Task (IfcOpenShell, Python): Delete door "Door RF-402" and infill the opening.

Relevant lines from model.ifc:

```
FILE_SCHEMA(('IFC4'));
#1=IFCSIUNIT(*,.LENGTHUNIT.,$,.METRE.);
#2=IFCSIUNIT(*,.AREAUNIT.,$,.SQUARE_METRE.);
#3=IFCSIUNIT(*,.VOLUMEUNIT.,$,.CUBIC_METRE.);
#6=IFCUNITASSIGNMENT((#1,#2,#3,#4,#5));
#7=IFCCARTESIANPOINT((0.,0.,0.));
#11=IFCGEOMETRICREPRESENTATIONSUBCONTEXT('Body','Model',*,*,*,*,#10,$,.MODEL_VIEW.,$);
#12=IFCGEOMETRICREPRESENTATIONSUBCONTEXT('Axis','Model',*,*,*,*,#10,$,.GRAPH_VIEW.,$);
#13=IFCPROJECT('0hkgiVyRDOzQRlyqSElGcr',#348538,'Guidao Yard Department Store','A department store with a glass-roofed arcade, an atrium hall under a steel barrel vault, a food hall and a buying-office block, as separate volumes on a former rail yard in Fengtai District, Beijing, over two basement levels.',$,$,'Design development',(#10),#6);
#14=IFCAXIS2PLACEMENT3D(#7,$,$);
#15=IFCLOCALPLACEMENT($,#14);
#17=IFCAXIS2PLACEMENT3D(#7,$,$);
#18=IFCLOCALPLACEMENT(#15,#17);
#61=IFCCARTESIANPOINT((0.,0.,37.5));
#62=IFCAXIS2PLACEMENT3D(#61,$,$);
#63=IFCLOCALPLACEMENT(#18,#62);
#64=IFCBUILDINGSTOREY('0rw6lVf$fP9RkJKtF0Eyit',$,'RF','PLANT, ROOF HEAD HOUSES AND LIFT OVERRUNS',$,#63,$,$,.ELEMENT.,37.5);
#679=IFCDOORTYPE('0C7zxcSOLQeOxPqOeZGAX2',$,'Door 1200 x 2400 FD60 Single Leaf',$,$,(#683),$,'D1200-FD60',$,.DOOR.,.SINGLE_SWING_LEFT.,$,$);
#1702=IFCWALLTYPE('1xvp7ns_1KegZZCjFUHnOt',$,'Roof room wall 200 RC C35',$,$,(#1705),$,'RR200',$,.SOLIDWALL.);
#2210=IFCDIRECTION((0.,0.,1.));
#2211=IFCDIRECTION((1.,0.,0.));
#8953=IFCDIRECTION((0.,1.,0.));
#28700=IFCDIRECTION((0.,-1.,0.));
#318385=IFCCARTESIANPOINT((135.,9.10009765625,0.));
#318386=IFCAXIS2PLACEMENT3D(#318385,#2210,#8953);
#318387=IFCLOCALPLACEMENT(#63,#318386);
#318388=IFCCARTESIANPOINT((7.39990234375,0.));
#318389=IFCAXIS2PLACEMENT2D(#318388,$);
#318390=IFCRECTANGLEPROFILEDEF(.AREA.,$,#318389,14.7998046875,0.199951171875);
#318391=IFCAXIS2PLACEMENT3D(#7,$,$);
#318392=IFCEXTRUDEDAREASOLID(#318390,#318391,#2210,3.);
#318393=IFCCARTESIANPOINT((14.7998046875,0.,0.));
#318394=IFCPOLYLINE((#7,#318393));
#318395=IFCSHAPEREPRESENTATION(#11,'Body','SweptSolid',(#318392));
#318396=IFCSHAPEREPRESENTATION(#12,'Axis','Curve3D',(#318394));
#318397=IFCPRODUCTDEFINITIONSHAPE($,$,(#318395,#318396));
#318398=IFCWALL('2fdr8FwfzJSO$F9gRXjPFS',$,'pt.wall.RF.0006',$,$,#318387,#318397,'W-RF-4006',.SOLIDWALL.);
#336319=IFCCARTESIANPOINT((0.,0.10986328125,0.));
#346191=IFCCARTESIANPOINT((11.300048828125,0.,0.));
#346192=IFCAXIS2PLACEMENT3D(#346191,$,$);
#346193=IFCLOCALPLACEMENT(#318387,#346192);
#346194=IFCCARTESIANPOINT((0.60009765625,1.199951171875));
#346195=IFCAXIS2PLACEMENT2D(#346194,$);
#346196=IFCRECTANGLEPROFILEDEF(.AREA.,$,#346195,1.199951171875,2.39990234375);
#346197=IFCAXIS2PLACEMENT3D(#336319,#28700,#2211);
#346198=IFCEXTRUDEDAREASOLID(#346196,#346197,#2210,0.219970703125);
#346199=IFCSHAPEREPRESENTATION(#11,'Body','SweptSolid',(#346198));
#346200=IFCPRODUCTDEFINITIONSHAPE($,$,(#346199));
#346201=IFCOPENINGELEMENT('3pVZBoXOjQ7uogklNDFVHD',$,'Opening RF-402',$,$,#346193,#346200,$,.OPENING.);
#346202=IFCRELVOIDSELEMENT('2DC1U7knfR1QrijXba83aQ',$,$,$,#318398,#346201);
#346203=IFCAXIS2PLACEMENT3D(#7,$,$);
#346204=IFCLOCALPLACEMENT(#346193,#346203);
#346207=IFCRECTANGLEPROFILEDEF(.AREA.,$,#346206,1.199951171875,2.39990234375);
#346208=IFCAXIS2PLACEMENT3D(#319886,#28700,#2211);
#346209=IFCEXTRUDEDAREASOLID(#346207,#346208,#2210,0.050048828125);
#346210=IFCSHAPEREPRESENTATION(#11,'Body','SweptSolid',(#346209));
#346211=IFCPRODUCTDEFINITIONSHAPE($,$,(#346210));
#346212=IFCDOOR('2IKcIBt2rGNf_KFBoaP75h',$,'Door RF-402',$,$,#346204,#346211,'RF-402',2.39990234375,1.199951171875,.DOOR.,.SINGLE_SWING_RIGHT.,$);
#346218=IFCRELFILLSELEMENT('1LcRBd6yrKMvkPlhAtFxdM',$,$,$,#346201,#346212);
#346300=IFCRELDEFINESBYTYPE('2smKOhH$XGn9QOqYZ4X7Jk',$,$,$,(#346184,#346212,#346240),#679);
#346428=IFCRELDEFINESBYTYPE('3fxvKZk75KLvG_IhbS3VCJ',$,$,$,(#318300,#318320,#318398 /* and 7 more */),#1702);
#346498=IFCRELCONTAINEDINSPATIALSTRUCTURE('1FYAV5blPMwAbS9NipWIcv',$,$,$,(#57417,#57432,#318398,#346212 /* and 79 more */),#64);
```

```python
import ifcopenshell
import ifcopenshell.api.feature
import ifcopenshell.api.root
import ifcopenshell.geom
import ifcopenshell.util.shape

model = ifcopenshell.open("model.ifc")
settings = ifcopenshell.geom.settings()


def volume(element):
    """Net volume in cubic metres, openings subtracted."""
    shape = ifcopenshell.geom.create_shape(settings, element)
    return ifcopenshell.util.shape.get_volume(shape.geometry)


door = model.by_guid("2IKcIBt2rGNf_KFBoaP75h")
opening = door.FillsVoids[0].RelatingOpeningElement
wall = opening.VoidsElements[0].RelatingBuildingElement
before = volume(wall)

ifcopenshell.api.root.remove_product(model, product=door)
ifcopenshell.api.feature.remove_feature(model, feature=opening)

after = volume(wall)

print(f"wall volume {before:.3f} -> {after:.3f} m3")

model.write("model_updated.ifc")
```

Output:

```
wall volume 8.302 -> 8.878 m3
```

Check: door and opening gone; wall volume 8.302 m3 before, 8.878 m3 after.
